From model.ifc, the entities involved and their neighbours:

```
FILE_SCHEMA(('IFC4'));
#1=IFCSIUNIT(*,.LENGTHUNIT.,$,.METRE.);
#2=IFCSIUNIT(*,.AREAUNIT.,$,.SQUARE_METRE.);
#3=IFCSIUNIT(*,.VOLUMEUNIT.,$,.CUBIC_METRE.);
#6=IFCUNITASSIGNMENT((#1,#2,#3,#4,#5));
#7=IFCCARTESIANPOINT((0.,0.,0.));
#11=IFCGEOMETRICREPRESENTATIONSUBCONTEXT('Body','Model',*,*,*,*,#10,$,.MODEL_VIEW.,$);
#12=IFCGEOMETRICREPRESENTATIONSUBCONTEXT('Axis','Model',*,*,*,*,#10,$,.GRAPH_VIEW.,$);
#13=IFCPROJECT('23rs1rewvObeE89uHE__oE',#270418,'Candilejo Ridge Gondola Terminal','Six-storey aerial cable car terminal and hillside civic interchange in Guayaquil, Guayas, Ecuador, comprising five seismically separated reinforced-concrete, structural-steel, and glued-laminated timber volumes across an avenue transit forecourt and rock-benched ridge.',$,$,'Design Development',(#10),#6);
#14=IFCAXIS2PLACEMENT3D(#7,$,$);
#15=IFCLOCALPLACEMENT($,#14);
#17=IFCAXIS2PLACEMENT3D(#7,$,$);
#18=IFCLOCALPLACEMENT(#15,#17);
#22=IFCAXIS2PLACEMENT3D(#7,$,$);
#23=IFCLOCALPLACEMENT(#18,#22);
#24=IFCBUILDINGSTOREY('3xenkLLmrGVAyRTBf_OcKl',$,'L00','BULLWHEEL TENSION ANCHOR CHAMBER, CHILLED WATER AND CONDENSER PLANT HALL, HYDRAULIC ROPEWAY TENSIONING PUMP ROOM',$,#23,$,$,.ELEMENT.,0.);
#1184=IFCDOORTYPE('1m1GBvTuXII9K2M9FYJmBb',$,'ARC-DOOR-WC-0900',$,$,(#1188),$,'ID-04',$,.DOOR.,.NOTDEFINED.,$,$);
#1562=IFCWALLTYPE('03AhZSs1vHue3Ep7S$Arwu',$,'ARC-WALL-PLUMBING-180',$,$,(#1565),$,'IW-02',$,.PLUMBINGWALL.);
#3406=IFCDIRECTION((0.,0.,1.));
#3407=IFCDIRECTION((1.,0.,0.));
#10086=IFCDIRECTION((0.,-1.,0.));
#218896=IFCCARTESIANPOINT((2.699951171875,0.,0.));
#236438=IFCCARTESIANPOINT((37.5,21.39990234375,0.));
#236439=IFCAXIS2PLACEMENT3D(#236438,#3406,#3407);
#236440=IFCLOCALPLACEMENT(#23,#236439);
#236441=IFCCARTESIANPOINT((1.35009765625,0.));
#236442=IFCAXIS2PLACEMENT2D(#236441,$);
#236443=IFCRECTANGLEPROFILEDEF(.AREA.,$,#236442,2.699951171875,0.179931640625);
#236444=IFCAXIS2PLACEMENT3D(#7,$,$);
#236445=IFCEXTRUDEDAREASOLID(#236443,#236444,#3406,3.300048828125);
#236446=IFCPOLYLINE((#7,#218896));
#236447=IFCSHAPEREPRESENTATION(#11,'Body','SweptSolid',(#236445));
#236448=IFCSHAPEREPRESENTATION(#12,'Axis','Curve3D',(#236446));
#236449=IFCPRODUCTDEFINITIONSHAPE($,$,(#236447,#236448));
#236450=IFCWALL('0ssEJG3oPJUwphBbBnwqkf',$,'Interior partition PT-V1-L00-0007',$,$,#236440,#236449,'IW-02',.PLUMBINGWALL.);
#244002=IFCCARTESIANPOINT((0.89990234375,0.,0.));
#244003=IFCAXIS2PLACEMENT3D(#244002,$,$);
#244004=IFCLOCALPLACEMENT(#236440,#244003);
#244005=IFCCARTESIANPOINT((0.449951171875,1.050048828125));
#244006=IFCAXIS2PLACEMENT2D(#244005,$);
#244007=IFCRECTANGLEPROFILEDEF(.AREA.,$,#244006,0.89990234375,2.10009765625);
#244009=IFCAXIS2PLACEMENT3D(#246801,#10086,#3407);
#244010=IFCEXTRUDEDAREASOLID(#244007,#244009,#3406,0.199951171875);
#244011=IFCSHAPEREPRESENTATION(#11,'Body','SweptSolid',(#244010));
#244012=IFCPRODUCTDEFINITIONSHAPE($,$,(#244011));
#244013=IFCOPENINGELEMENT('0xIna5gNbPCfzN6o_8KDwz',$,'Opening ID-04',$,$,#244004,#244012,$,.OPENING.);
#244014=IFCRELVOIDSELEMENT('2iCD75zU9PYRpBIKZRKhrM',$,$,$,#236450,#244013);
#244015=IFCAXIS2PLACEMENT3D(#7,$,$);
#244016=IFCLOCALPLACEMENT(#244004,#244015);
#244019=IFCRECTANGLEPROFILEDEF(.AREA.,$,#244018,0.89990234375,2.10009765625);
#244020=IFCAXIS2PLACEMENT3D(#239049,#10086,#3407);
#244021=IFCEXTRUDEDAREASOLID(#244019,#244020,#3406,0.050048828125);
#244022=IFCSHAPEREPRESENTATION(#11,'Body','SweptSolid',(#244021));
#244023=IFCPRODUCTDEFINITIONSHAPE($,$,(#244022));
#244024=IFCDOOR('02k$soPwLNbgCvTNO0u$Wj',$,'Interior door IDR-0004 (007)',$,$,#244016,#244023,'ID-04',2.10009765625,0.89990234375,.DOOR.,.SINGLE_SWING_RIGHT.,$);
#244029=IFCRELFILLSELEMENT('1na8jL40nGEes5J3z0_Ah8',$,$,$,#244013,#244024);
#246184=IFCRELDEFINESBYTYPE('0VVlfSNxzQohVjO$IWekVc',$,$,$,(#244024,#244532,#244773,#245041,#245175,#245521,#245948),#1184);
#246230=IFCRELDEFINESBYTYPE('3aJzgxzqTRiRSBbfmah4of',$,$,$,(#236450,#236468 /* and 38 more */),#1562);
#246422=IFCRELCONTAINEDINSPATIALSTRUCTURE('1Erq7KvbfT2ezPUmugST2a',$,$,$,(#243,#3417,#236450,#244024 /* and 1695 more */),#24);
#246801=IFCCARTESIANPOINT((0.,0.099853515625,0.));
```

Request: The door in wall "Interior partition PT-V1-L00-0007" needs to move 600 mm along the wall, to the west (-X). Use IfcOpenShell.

```python
import ifcopenshell
import ifcopenshell.api.geometry
import ifcopenshell.util.placement
import ifcopenshell.util.unit

model = ifcopenshell.open("model.ifc")
unit_scale = ifcopenshell.util.unit.calculate_unit_scale(model)

door = model.by_guid("02k$soPwLNbgCvTNO0u$Wj")
opening = door.FillsVoids[0].RelatingOpeningElement
wall = opening.VoidsElements[0].RelatingBuildingElement

wall_matrix = ifcopenshell.util.placement.get_local_placement(wall.ObjectPlacement)
shift = wall_matrix[:3, 0] * -0.6 / unit_scale
before = ifcopenshell.util.placement.get_local_placement(door.ObjectPlacement)[:3, 3].copy()

# The door is placed relative to its opening, so it follows when the opening moves.
matrix = ifcopenshell.util.placement.get_local_placement(opening.ObjectPlacement)
matrix[:3, 3] += shift
ifcopenshell.api.geometry.edit_object_placement(
    model, product=opening, matrix=matrix, is_si=False, should_transform_children=True
)

after = ifcopenshell.util.placement.get_local_placement(door.ObjectPlacement)[:3, 3]
print("door moved by", (after - before).round(3) + 0.0)

model.write("model_rev.ifc")
```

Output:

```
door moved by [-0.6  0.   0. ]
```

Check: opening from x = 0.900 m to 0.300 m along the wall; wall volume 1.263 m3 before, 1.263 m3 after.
